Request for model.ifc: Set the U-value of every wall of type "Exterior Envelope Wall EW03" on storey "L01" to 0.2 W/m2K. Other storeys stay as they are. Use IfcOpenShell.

First a look at what the model holds.

```python
import ifcopenshell
import ifcopenshell.util.element

model = ifcopenshell.open("model.ifc")
print(model.schema)
storey = next(s for s in model.by_type("IfcBuildingStorey") if s.Name == "L01")
walls = [e for e in ifcopenshell.util.element.get_decomposition(storey) if e.is_a("IfcWall")]
seen = {}
for e in walls:
    element_type = ifcopenshell.util.element.get_type(e)
    key = (element_type.Name if element_type != e and element_type else None, ifcopenshell.util.element.get_pset(e, "Pset_WallCommon", "ThermalTransmittance"))
    seen[key] = seen.get(key, 0) + 1
for (name, value), count in sorted(seen.items(), key=str):
    print(count, "x", name, "|", value)
```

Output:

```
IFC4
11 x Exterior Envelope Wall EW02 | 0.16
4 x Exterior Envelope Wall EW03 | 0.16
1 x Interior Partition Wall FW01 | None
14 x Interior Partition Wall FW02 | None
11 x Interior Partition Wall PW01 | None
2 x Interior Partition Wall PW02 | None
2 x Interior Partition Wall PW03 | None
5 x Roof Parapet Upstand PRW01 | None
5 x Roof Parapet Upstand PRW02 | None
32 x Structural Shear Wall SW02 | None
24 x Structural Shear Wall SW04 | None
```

```python
import ifcopenshell
import ifcopenshell.api.pset
import ifcopenshell.util.element

model = ifcopenshell.open("model.ifc")

storey = next(s for s in model.by_type("IfcBuildingStorey") if s.Name == "L01")
walls = [e for e in ifcopenshell.util.element.get_decomposition(storey) if e.is_a("IfcWall")]

count = 0
for e in walls:
    element_type = ifcopenshell.util.element.get_type(e)
    if element_type in (None, e) or element_type.Name != "Exterior Envelope Wall EW03":
        continue
    # add_pset returns the element's existing set when there is one.
    pset = ifcopenshell.api.pset.add_pset(model, product=e, name="Pset_WallCommon")
    ifcopenshell.api.pset.edit_pset(model, pset=pset, properties={"ThermalTransmittance": 0.2})
    count += 1

print(count, "walls updated")

model.write("model_updated.ifc")
```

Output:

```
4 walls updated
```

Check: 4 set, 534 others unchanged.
